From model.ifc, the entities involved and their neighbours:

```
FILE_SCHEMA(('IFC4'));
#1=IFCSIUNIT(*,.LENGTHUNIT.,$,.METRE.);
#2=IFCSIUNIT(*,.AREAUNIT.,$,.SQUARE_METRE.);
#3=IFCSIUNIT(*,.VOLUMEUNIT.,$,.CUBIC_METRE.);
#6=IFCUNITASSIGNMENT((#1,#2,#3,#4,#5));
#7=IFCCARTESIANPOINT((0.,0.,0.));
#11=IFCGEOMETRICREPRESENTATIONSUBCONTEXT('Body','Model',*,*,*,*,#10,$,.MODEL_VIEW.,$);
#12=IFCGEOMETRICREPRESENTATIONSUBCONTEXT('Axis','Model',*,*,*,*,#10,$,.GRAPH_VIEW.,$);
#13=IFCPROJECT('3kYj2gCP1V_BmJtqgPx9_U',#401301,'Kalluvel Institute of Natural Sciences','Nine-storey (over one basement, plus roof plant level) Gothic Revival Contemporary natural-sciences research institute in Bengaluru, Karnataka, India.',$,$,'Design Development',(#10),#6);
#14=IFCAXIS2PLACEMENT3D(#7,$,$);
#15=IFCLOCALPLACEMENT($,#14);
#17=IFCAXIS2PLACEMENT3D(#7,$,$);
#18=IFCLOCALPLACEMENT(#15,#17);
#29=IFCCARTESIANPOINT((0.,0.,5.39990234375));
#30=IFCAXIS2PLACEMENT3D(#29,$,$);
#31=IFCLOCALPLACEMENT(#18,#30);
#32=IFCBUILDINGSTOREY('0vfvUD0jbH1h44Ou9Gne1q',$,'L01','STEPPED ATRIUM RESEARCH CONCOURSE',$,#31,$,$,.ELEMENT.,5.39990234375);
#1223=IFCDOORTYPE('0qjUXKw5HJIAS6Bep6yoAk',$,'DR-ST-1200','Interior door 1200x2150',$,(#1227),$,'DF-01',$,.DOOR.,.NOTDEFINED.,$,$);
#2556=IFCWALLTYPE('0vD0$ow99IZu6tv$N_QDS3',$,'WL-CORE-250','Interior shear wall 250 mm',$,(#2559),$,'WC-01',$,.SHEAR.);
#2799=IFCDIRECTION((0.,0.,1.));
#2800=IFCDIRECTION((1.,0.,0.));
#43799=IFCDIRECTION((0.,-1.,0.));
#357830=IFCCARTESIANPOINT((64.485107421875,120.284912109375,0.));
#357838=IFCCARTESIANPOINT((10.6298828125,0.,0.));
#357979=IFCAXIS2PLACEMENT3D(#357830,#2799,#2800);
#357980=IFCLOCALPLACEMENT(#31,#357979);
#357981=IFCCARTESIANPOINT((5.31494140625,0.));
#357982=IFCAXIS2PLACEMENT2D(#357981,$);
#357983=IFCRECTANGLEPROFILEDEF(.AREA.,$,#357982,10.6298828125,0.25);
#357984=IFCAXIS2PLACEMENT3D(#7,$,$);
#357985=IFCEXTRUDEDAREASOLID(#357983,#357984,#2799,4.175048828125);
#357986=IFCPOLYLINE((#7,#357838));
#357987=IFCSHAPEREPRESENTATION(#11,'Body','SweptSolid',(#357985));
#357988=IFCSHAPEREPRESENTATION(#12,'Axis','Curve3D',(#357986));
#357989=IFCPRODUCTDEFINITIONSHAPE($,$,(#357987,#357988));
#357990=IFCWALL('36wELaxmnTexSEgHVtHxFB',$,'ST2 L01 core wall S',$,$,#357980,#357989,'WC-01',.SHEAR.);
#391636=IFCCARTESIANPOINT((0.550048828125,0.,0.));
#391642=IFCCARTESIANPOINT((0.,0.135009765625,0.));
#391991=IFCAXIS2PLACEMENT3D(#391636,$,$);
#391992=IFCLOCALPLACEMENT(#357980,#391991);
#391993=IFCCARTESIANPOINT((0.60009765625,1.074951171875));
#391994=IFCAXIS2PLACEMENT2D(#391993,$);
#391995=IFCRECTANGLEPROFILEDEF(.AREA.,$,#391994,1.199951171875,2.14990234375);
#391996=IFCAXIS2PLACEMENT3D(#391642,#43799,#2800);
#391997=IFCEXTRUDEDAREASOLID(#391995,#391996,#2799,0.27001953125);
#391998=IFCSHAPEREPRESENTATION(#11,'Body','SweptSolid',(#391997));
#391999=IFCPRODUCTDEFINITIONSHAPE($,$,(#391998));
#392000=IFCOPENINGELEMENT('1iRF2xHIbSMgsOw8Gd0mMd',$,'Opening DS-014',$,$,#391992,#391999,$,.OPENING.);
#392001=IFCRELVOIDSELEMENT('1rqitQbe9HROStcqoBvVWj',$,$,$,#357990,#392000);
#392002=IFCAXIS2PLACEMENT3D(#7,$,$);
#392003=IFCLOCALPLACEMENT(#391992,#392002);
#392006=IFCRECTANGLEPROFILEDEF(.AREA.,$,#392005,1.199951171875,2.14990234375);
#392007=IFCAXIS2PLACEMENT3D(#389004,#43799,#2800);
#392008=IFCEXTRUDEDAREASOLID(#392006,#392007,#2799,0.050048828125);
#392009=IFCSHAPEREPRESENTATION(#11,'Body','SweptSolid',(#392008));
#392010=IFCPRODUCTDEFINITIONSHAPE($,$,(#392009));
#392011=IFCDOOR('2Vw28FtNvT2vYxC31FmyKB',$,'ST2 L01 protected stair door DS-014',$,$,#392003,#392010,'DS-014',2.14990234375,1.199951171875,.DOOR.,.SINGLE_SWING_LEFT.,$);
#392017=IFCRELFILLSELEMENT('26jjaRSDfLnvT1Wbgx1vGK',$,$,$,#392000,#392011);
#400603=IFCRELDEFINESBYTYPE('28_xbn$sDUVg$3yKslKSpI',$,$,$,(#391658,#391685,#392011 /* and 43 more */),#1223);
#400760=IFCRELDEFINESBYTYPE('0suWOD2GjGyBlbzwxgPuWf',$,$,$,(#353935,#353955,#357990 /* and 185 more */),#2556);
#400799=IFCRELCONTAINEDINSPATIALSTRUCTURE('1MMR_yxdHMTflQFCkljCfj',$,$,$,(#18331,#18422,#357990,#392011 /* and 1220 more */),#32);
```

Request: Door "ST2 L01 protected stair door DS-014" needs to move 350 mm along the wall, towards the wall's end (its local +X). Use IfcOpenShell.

```python
import ifcopenshell
import ifcopenshell.api.geometry
import ifcopenshell.util.placement
import ifcopenshell.util.unit

model = ifcopenshell.open("model.ifc")
unit_scale = ifcopenshell.util.unit.calculate_unit_scale(model)

door = model.by_guid("2Vw28FtNvT2vYxC31FmyKB")
opening = door.FillsVoids[0].RelatingOpeningElement
wall = opening.VoidsElements[0].RelatingBuildingElement

wall_matrix = ifcopenshell.util.placement.get_local_placement(wall.ObjectPlacement)
shift = wall_matrix[:3, 0] * 0.35 / unit_scale
before = ifcopenshell.util.placement.get_local_placement(door.ObjectPlacement)[:3, 3].copy()

# The door is placed relative to its opening, so it follows when the opening moves.
matrix = ifcopenshell.util.placement.get_local_placement(opening.ObjectPlacement)
matrix[:3, 3] += shift
ifcopenshell.api.geometry.edit_object_placement(
    model, product=opening, matrix=matrix, is_si=False, should_transform_children=True
)

after = ifcopenshell.util.placement.get_local_placement(door.ObjectPlacement)[:3, 3]
print("door moved by", (after - before).round(3) + 0.0)

model.write("model_v2.ifc")
```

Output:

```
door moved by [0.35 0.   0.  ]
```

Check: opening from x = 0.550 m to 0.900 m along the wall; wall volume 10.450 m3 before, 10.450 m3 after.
